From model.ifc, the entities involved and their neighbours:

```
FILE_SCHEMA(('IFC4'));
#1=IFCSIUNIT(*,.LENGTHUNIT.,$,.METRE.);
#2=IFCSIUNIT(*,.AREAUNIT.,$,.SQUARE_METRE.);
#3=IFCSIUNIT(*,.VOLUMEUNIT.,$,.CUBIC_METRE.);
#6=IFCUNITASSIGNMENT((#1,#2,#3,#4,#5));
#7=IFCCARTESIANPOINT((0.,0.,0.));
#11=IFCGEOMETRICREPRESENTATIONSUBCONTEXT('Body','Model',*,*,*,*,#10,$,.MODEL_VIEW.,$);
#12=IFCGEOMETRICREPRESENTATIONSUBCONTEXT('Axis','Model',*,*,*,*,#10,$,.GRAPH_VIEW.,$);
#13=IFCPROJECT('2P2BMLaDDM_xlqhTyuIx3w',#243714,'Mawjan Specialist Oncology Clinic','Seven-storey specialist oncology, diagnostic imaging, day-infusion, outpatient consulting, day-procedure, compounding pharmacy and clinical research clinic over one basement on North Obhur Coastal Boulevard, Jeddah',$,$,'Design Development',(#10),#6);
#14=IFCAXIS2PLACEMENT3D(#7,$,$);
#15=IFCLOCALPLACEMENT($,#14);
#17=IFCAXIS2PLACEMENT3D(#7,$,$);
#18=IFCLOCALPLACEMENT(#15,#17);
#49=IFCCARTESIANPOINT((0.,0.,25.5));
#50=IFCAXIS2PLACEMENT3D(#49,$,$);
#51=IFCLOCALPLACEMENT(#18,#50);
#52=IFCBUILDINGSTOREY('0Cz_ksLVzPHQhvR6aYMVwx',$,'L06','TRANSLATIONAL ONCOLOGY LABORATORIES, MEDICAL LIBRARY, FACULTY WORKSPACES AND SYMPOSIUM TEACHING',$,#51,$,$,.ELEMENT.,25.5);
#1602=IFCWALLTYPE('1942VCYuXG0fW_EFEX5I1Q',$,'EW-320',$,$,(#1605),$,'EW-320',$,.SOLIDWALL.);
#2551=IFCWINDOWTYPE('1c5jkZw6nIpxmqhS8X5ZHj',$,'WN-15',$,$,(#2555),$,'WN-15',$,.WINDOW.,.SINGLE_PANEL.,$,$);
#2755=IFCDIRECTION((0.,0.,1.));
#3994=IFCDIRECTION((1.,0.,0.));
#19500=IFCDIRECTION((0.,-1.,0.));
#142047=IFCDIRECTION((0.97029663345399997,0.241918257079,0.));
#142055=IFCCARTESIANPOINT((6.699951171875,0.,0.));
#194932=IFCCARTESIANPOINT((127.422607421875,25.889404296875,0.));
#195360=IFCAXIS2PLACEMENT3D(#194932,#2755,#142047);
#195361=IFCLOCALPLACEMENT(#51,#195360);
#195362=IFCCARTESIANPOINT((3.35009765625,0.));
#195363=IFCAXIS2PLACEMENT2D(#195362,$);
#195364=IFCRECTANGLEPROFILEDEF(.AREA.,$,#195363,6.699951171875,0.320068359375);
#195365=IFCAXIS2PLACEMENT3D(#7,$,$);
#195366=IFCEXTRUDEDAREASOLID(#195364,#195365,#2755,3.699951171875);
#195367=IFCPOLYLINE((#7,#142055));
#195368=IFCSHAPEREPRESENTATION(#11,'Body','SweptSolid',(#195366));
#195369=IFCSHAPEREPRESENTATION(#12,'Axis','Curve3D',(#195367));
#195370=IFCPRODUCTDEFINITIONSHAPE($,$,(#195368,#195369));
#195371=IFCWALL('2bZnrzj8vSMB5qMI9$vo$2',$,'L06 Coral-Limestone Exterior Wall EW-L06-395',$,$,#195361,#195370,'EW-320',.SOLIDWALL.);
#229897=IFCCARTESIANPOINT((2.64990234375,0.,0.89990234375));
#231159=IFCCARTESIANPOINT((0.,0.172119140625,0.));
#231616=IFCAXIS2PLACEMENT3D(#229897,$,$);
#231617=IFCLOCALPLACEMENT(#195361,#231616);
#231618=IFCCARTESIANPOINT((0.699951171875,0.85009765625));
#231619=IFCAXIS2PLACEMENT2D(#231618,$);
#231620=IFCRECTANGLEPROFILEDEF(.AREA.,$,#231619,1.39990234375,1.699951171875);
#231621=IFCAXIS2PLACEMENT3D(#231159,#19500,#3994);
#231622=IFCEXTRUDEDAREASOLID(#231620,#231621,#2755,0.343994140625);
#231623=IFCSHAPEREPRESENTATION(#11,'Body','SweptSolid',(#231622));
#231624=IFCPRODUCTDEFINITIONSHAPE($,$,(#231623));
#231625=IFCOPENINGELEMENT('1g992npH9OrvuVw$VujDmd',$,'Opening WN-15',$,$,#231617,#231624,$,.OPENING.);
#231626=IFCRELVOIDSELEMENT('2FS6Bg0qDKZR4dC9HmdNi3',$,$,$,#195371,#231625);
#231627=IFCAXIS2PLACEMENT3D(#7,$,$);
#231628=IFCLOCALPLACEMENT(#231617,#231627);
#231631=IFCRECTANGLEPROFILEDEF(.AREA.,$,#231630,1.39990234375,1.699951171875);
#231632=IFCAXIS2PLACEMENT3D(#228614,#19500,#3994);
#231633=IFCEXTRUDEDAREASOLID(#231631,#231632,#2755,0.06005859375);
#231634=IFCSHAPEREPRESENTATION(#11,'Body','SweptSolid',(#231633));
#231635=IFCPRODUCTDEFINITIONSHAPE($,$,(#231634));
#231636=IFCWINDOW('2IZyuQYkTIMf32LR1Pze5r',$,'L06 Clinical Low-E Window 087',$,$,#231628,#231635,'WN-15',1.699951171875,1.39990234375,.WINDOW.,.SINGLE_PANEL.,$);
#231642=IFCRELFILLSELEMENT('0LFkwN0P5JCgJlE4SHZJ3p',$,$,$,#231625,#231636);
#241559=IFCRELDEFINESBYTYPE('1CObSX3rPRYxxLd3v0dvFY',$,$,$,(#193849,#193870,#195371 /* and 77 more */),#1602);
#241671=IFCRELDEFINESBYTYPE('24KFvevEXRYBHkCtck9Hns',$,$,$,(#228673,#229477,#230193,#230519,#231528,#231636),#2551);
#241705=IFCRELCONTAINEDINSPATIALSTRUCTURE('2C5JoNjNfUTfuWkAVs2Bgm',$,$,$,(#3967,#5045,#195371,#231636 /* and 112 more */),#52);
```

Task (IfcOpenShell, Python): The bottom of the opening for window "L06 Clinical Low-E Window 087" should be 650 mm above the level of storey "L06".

```python
import numpy as np
import ifcopenshell
import ifcopenshell.api.geometry
import ifcopenshell.geom
import ifcopenshell.util.element
import ifcopenshell.util.placement
import ifcopenshell.util.shape
import ifcopenshell.util.unit

model = ifcopenshell.open("model.ifc")
unit_scale = ifcopenshell.util.unit.calculate_unit_scale(model)

window = model.by_guid("2IZyuQYkTIMf32LR1Pze5r")
opening = window.FillsVoids[0].RelatingOpeningElement
storey = ifcopenshell.util.element.get_container(window, ifc_class="IfcBuildingStorey")
level = ifcopenshell.util.placement.get_local_placement(storey.ObjectPlacement)[2, 3]

# The opening's origin need not be at the sill, so measure its lowest point.
shape = ifcopenshell.geom.create_shape(ifcopenshell.geom.settings(), opening)
bottom = ifcopenshell.util.shape.get_shape_bottom_elevation(shape, shape.geometry) / unit_scale
dz = level + 0.65 - bottom

shift = np.array([0.0, 0.0, dz])
# The window is placed relative to its opening, so it follows when the opening moves.
matrix = ifcopenshell.util.placement.get_local_placement(opening.ObjectPlacement)
matrix[:3, 3] += shift
ifcopenshell.api.geometry.edit_object_placement(
    model, product=opening, matrix=matrix, is_si=False, should_transform_children=True
)

print(f"moved by {dz * unit_scale:+.3f} m")

model.write("model-out.ifc")
```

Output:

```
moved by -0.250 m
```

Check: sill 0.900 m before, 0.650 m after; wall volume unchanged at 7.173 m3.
